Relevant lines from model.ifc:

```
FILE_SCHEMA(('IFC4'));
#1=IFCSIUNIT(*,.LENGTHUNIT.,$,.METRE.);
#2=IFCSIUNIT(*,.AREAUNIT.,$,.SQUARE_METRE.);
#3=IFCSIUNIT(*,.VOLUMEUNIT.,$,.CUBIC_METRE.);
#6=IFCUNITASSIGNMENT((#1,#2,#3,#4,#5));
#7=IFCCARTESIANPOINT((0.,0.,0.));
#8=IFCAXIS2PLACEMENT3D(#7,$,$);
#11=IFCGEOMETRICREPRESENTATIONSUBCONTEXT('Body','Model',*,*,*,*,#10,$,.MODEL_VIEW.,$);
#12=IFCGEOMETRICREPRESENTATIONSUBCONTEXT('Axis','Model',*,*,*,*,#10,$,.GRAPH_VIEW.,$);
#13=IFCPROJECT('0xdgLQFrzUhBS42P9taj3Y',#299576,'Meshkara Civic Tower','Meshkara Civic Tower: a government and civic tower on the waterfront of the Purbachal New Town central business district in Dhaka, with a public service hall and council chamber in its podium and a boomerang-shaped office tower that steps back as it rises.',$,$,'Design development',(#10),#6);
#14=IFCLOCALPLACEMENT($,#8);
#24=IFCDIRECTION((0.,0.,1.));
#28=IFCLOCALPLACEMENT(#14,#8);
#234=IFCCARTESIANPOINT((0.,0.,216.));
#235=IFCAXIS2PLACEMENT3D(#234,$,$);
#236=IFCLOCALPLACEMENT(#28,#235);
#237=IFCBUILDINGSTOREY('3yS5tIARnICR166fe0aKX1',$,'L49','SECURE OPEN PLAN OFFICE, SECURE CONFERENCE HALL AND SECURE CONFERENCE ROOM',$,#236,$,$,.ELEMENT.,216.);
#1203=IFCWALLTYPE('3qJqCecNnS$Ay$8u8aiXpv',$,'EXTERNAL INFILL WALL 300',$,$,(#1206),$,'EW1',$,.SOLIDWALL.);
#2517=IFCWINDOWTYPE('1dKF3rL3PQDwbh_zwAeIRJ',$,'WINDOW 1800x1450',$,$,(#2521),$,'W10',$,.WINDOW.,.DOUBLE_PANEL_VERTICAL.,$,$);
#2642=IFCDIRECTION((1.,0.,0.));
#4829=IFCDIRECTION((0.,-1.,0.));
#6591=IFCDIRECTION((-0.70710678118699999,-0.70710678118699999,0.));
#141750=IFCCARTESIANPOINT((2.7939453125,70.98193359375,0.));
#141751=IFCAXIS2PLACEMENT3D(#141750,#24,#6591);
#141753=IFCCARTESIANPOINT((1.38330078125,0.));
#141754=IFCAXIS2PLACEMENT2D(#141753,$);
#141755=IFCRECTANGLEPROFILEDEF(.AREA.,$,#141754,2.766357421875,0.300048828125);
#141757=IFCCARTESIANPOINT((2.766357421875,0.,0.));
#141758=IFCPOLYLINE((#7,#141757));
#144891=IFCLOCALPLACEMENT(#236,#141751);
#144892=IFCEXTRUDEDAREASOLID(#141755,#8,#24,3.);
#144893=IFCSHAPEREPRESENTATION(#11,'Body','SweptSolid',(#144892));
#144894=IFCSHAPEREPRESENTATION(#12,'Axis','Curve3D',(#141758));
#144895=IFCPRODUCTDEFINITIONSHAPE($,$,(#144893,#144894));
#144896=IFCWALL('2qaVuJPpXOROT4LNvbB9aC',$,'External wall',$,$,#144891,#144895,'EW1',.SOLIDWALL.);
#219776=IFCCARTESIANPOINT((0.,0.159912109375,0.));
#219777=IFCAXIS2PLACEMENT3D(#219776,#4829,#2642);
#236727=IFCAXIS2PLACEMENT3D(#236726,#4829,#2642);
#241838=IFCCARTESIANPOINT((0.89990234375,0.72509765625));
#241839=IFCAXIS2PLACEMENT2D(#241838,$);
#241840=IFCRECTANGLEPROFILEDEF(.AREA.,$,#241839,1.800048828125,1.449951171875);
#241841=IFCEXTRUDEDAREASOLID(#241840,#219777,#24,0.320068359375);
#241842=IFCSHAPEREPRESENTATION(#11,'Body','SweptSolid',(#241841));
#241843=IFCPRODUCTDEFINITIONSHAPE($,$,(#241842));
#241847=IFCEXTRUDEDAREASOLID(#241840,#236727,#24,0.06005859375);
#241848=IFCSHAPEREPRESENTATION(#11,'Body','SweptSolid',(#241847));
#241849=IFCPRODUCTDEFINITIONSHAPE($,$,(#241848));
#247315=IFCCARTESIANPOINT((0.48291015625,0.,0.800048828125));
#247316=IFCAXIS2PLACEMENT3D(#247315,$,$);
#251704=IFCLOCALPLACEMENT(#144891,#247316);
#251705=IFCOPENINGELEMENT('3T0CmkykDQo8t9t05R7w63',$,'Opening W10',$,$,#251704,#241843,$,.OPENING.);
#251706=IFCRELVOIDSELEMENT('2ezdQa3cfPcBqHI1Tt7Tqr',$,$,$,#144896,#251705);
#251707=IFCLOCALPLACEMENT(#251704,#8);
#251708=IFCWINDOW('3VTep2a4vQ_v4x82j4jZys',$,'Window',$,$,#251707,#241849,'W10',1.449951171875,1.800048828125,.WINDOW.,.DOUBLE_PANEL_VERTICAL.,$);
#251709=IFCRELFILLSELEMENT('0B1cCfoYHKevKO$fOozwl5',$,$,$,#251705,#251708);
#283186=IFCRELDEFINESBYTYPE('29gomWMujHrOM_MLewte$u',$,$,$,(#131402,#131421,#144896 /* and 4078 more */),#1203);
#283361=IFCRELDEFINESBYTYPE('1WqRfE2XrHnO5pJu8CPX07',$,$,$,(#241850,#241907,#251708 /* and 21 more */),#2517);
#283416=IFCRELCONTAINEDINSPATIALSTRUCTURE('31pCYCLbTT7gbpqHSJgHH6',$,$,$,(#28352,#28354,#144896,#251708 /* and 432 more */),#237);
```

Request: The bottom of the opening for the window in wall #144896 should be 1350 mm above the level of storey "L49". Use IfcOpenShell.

```python
import numpy as np
import ifcopenshell
import ifcopenshell.api.geometry
import ifcopenshell.geom
import ifcopenshell.util.element
import ifcopenshell.util.placement
import ifcopenshell.util.shape
import ifcopenshell.util.unit

model = ifcopenshell.open("model.ifc")
unit_scale = ifcopenshell.util.unit.calculate_unit_scale(model)

window = model.by_guid("3VTep2a4vQ_v4x82j4jZys")
opening = window.FillsVoids[0].RelatingOpeningElement
storey = ifcopenshell.util.element.get_container(window, ifc_class="IfcBuildingStorey")
level = ifcopenshell.util.placement.get_local_placement(storey.ObjectPlacement)[2, 3]

# The opening's origin need not be at the sill, so measure its lowest point.
shape = ifcopenshell.geom.create_shape(ifcopenshell.geom.settings(), opening)
bottom = ifcopenshell.util.shape.get_shape_bottom_elevation(shape, shape.geometry) / unit_scale
dz = level + 1.35 - bottom

shift = np.array([0.0, 0.0, dz])
# The window is placed relative to its opening, so it follows when the opening moves.
matrix = ifcopenshell.util.placement.get_local_placement(opening.ObjectPlacement)
matrix[:3, 3] += shift
ifcopenshell.api.geometry.edit_object_placement(
    model, product=opening, matrix=matrix, is_si=False, should_transform_children=True
)

print(f"moved by {dz * unit_scale:+.3f} m")

model.write("model_updated.ifc")
```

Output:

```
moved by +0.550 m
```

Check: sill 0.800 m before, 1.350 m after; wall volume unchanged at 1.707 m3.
